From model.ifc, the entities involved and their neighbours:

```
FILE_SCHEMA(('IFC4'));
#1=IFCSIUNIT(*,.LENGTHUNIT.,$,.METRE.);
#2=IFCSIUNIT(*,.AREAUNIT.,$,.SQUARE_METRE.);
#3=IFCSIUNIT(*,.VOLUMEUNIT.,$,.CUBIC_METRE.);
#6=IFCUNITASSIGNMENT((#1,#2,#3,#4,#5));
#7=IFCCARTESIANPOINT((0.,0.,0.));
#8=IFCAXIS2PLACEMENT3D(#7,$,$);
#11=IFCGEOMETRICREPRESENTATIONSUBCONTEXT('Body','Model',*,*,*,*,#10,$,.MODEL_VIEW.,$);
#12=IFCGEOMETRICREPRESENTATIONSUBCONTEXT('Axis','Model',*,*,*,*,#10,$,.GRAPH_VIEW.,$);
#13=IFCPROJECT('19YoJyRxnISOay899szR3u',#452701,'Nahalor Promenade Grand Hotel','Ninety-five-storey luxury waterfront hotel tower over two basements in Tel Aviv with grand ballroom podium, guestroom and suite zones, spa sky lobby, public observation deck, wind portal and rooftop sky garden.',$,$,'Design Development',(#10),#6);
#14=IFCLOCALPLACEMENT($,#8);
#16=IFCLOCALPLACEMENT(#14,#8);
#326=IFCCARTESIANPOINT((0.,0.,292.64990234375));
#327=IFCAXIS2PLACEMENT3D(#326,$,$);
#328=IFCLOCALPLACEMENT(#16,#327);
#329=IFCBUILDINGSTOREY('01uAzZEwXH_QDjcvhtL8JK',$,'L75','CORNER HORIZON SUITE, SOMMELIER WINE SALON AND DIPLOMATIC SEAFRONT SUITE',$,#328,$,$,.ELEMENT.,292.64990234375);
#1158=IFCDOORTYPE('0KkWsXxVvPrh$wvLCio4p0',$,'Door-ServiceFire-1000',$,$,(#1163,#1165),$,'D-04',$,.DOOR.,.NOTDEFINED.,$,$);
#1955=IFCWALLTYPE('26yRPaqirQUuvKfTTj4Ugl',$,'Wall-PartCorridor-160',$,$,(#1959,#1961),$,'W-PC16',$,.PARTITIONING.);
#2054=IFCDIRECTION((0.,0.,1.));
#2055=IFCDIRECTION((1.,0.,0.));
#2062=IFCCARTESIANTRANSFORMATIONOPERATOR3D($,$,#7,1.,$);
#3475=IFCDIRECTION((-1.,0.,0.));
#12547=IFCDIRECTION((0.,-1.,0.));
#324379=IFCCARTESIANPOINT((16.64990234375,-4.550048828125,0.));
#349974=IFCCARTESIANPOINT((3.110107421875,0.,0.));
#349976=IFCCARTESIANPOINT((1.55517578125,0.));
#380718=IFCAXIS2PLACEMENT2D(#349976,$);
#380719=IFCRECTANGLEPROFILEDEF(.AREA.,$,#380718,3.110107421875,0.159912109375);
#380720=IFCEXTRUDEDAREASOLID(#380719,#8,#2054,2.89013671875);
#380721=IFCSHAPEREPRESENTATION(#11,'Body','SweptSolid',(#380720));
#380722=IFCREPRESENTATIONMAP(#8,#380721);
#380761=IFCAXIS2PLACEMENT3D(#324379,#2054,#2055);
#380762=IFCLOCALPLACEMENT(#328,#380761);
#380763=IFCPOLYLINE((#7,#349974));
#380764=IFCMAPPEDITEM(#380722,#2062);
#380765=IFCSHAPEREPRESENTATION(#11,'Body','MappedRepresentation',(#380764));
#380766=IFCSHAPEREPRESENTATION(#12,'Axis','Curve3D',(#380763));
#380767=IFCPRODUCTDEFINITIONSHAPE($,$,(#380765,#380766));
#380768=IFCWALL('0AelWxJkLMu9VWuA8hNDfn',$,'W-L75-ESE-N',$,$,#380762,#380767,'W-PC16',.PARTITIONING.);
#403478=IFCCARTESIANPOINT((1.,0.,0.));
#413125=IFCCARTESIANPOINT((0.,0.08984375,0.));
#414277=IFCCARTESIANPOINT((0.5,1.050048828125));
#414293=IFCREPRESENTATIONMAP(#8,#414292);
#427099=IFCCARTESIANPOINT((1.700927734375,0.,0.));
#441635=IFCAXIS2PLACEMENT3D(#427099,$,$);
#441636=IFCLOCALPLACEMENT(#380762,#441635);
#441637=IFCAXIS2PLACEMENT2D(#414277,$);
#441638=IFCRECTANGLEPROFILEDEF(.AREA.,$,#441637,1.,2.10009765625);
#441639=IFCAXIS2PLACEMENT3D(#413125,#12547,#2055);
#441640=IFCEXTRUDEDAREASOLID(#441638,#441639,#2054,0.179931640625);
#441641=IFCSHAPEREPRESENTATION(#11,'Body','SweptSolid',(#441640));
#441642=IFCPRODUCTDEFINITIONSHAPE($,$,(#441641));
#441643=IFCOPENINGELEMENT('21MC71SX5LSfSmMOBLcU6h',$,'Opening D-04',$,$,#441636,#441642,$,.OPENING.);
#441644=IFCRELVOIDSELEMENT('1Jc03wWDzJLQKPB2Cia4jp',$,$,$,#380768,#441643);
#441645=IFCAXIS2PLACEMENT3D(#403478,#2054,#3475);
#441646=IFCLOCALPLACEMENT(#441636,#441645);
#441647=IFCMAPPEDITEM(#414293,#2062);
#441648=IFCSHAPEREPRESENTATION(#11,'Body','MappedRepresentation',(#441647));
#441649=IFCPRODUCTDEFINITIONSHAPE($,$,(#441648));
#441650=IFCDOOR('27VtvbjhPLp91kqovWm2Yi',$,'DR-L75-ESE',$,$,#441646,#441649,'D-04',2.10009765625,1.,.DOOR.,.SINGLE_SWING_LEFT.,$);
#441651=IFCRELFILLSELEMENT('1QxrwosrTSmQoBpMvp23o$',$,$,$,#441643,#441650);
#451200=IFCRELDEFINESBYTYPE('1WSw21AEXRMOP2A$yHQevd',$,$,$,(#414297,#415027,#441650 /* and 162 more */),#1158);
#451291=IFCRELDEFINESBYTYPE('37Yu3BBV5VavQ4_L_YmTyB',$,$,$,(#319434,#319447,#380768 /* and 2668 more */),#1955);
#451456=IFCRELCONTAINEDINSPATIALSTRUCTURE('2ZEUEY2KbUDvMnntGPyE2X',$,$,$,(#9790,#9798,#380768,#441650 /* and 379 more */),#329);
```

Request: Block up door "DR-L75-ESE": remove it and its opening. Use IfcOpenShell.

```python
import ifcopenshell
import ifcopenshell.api.feature
import ifcopenshell.api.root
import ifcopenshell.geom
import ifcopenshell.util.shape

model = ifcopenshell.open("model.ifc")
settings = ifcopenshell.geom.settings()


def volume(element):
    """Net volume in cubic metres, openings subtracted."""
    shape = ifcopenshell.geom.create_shape(settings, element)
    return ifcopenshell.util.shape.get_volume(shape.geometry)


door = model.by_guid("27VtvbjhPLp91kqovWm2Yi")
opening = door.FillsVoids[0].RelatingOpeningElement
wall = opening.VoidsElements[0].RelatingBuildingElement
before = volume(wall)

ifcopenshell.api.root.remove_product(model, product=door)
ifcopenshell.api.feature.remove_feature(model, feature=opening)

after = volume(wall)

print(f"wall volume {before:.3f} -> {after:.3f} m3")

model.write("model_v2.ifc")
```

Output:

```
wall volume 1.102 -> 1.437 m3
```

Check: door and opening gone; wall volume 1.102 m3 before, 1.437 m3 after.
